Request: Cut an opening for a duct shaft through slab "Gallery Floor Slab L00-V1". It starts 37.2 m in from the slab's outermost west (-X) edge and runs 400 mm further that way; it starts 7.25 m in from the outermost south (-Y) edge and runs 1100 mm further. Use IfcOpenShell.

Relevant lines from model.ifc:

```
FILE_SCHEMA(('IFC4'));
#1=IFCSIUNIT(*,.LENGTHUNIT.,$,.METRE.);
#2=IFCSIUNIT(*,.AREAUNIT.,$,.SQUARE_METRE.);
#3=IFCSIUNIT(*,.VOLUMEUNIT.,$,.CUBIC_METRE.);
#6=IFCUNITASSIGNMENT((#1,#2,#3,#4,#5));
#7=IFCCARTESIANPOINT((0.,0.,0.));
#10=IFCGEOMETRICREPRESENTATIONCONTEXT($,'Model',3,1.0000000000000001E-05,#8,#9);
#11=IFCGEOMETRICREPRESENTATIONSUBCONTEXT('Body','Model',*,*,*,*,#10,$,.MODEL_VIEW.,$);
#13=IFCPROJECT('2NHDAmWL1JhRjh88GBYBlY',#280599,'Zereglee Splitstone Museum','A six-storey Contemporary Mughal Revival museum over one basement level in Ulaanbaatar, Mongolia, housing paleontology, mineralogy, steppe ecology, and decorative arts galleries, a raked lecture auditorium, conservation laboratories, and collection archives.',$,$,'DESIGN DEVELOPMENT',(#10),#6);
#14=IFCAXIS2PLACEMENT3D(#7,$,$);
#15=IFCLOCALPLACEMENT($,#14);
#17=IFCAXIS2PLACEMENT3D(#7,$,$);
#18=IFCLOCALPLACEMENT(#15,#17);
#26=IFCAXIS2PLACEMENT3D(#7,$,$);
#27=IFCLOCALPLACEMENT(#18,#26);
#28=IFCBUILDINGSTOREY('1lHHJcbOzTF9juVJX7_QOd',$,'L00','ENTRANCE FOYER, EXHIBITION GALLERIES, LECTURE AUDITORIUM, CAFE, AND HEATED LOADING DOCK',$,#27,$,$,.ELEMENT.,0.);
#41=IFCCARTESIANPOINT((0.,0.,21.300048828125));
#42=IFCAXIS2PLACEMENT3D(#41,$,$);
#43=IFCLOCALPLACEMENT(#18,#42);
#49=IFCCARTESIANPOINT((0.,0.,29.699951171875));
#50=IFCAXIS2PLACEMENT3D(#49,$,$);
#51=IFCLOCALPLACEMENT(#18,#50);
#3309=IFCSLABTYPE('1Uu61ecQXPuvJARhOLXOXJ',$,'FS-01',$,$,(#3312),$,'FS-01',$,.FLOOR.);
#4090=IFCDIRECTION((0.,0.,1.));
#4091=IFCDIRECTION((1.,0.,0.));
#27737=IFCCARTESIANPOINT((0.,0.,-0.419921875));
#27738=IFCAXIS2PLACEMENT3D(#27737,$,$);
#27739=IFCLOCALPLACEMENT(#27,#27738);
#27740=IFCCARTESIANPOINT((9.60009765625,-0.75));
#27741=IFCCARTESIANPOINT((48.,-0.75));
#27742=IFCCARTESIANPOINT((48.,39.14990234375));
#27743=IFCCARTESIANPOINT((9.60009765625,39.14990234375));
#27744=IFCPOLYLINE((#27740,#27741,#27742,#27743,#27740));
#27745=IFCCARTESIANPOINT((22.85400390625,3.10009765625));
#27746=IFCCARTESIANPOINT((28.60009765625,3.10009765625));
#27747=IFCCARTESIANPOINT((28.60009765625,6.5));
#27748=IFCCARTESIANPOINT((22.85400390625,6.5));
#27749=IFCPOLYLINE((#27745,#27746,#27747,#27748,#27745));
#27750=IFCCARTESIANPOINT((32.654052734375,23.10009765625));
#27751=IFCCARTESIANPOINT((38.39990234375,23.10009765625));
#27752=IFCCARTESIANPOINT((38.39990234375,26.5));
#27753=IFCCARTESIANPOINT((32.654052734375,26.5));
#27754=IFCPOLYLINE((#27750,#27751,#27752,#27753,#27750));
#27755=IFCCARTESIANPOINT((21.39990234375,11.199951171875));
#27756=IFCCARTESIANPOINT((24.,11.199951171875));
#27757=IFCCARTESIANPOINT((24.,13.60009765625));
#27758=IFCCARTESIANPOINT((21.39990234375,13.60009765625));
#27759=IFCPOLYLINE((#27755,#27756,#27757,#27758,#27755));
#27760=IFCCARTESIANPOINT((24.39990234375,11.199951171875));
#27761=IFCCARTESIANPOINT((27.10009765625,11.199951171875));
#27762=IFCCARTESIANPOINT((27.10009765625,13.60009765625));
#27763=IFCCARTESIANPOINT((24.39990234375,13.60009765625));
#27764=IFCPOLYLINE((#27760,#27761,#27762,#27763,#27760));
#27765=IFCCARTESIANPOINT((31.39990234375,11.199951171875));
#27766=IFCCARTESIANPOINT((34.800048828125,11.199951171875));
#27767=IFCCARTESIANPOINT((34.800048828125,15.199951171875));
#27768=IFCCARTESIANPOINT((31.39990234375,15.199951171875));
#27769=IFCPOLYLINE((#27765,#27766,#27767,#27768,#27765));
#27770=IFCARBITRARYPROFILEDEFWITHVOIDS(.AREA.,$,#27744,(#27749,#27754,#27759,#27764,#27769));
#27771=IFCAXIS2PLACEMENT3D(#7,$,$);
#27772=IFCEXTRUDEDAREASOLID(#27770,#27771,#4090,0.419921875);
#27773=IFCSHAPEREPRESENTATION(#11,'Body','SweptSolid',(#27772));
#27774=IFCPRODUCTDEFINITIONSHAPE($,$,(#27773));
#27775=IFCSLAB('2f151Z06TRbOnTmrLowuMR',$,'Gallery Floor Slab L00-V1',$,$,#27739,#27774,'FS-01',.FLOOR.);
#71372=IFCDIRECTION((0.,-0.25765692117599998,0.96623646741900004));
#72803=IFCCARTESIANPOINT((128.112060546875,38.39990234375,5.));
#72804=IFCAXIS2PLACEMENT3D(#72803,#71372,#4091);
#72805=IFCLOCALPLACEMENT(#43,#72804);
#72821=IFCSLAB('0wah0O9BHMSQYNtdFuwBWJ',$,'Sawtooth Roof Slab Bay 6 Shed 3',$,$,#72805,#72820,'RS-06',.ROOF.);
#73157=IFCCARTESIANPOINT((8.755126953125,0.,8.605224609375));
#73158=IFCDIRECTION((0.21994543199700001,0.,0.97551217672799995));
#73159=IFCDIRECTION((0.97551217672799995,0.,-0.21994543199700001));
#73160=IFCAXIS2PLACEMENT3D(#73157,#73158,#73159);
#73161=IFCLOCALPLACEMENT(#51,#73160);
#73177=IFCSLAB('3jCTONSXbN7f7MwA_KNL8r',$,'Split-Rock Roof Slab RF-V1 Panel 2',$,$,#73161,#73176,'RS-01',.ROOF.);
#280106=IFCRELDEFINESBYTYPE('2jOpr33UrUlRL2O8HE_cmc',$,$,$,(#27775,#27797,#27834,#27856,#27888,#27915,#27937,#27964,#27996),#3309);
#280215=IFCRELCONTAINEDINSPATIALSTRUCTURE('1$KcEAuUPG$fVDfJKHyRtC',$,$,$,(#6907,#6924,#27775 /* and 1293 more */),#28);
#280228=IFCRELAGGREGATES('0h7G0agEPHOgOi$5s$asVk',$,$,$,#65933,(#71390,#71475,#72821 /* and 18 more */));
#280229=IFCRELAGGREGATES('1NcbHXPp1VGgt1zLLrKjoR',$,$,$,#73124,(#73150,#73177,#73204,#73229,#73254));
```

```python
import numpy as np
import ifcopenshell
import ifcopenshell.api.feature
import ifcopenshell.api.geometry
import ifcopenshell.api.root
import ifcopenshell.geom
import ifcopenshell.util.placement
import ifcopenshell.util.representation
import ifcopenshell.util.shape
import ifcopenshell.util.unit

model = ifcopenshell.open("model.ifc")
unit_scale = ifcopenshell.util.unit.calculate_unit_scale(model)
settings = ifcopenshell.geom.settings()


def volume(element):
    """Net volume in cubic metres, openings subtracted."""
    shape = ifcopenshell.geom.create_shape(settings, element)
    return ifcopenshell.util.shape.get_volume(shape.geometry)


slab = model.by_guid("2f151Z06TRbOnTmrLowuMR")
before = volume(slab)

# Extent in the slab's own axes, in metres. The edges named are its -X and -Y sides.
slab_shape = ifcopenshell.geom.create_shape(settings, slab)
vertices = ifcopenshell.util.shape.get_vertices(slab_shape.geometry)
x_min, y_min, bottom = vertices.min(axis=0)
top = vertices[:, 2].max()

opening = ifcopenshell.api.root.create_entity(model, ifc_class="IfcOpeningElement", name="Duct shaft opening", predefined_type="OPENING")
context = ifcopenshell.util.representation.get_context(model, "Model", "Body", "MODEL_VIEW")
width, depth = 0.4, 1.1
outline = [(0.0, 0.0), (width, 0.0), (width, depth), (0.0, depth), (0.0, 0.0)]
# Overshoot both faces by 50 mm so the cut is clean.
shape = ifcopenshell.api.geometry.add_slab_representation(
    model, context=context, depth=top - bottom + 0.1, polyline=outline
)
ifcopenshell.api.geometry.assign_representation(model, product=opening, representation=shape)

matrix = ifcopenshell.util.placement.get_local_placement(slab.ObjectPlacement)
matrix[:, 3] = matrix @ np.append(np.array([x_min + 37.2, y_min + 7.25, bottom - 0.05]) / unit_scale, 1.0)
ifcopenshell.api.geometry.edit_object_placement(model, product=opening, matrix=matrix, is_si=False)
ifcopenshell.api.feature.add_feature(model, feature=opening, element=slab)

after = volume(slab)

print(f"slab volume {before:.3f} -> {after:.3f} m3")

model.write("model_v2.ifc")
```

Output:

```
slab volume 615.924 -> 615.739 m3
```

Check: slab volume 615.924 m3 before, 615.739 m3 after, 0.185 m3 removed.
